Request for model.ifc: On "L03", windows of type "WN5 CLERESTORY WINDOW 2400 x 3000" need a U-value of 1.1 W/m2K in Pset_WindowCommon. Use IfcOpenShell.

First a look at what the model holds.

```python
import ifcopenshell
import ifcopenshell.util.element

model = ifcopenshell.open("model.ifc")
print(model.schema)
storey = next(s for s in model.by_type("IfcBuildingStorey") if s.Name == "L03")
windows = [e for e in ifcopenshell.util.element.get_decomposition(storey) if e.is_a("IfcWindow")]
seen = {}
for e in windows:
    element_type = ifcopenshell.util.element.get_type(e)
    key = (element_type.Name if element_type != e and element_type else None, ifcopenshell.util.element.get_pset(e, "Pset_WindowCommon", "ThermalTransmittance"))
    seen[key] = seen.get(key, 0) + 1
for (name, value), count in sorted(seen.items(), key=str):
    print(count, "x", name, "|", value)
```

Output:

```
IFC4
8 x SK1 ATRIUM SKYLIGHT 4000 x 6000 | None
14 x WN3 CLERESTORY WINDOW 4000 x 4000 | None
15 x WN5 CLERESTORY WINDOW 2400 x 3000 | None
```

```python
import ifcopenshell
import ifcopenshell.api.pset
import ifcopenshell.util.element

model = ifcopenshell.open("model.ifc")

storey = next(s for s in model.by_type("IfcBuildingStorey") if s.Name == "L03")
windows = [e for e in ifcopenshell.util.element.get_decomposition(storey) if e.is_a("IfcWindow")]

count = 0
for e in windows:
    element_type = ifcopenshell.util.element.get_type(e)
    if element_type in (None, e) or element_type.Name != "WN5 CLERESTORY WINDOW 2400 x 3000":
        continue
    found = ifcopenshell.util.element.get_pset(e, "Pset_WindowCommon", should_inherit=False)
    if found:
        pset = model.by_id(found["id"])
        if len(ifcopenshell.util.element.get_elements_by_pset(pset)) > 1:
            pset = ifcopenshell.api.pset.unshare_pset(model, products=[e], pset=pset)[0]
    else:
        pset = ifcopenshell.api.pset.add_pset(model, product=e, name="Pset_WindowCommon")
    ifcopenshell.api.pset.edit_pset(model, pset=pset, properties={"ThermalTransmittance": 1.1})
    count += 1

print(count, "windows updated")

model.write("model_rev.ifc")
```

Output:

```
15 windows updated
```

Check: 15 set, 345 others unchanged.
